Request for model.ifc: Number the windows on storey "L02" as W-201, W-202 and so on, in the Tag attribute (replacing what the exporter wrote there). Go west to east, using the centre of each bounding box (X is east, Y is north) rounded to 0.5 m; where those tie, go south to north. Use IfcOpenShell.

First a look at what the model holds.

```python
import ifcopenshell
import ifcopenshell.util.element
import ifcopenshell.util.placement

model = ifcopenshell.open("model.ifc")
print(model.schema)
storey = next(s for s in model.by_type("IfcBuildingStorey") if s.Name == "L02")
windows = [e for e in ifcopenshell.util.element.get_decomposition(storey) if e.is_a("IfcWindow")]
for e in sorted(windows, key=lambda e: e.id()):
    origin = ifcopenshell.util.placement.get_local_placement(e.ObjectPlacement)[:3, 3]
    print(e.id(), e.Tag, e.Name, origin.round(2) + 0.0, sep=" | ")
```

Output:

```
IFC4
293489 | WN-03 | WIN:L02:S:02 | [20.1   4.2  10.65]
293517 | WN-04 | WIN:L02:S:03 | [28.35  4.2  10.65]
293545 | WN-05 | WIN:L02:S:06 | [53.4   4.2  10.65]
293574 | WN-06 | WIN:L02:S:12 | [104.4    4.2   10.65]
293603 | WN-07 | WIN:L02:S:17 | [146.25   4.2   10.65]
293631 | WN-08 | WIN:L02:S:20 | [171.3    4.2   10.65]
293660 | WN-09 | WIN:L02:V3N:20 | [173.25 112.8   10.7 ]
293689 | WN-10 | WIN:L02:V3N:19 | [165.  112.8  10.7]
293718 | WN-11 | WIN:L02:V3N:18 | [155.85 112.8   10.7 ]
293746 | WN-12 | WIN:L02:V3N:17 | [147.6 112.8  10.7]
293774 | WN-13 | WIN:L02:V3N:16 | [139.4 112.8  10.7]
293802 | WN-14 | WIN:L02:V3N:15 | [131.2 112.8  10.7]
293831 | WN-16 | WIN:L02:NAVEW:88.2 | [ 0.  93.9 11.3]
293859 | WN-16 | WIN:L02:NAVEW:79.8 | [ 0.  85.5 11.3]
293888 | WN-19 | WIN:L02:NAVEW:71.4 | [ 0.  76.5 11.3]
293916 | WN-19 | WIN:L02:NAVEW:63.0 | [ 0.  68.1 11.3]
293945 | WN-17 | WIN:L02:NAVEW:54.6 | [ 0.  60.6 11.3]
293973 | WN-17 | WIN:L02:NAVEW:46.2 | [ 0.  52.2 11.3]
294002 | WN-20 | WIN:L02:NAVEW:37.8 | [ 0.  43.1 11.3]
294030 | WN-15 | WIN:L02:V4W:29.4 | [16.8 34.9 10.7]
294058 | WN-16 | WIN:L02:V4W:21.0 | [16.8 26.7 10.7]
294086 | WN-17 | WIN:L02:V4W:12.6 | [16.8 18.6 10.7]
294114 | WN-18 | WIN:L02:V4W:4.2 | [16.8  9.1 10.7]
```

```python
import ifcopenshell
import ifcopenshell.geom
import ifcopenshell.util.element
import ifcopenshell.util.shape

model = ifcopenshell.open("model.ifc")
settings = ifcopenshell.geom.settings()
settings.set("use-world-coords", True)


def centre(element):
    shape = ifcopenshell.geom.create_shape(settings, element)
    return ifcopenshell.util.shape.get_bbox_centroid(shape.geometry)


storey = next(s for s in model.by_type("IfcBuildingStorey") if s.Name == "L02")
windows = [e for e in ifcopenshell.util.element.get_decomposition(storey) if e.is_a("IfcWindow")]

# Insertion points can sit at a corner or the storey origin, so sort by the geometry (in metres).
centres = {e: centre(e) for e in windows}
windows.sort(key=lambda e: (round(centres[e][0] / 0.5), centres[e][1]))

for i, e in enumerate(windows, start=1):
    number = f"W-2{i:02d}"
    e.Tag = number
    print(e.id(), number)

model.write("model_v2.ifc")
```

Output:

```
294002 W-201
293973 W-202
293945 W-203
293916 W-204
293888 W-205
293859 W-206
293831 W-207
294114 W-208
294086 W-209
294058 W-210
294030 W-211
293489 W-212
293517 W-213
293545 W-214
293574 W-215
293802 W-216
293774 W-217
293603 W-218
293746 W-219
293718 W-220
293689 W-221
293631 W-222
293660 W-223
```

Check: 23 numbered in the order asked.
